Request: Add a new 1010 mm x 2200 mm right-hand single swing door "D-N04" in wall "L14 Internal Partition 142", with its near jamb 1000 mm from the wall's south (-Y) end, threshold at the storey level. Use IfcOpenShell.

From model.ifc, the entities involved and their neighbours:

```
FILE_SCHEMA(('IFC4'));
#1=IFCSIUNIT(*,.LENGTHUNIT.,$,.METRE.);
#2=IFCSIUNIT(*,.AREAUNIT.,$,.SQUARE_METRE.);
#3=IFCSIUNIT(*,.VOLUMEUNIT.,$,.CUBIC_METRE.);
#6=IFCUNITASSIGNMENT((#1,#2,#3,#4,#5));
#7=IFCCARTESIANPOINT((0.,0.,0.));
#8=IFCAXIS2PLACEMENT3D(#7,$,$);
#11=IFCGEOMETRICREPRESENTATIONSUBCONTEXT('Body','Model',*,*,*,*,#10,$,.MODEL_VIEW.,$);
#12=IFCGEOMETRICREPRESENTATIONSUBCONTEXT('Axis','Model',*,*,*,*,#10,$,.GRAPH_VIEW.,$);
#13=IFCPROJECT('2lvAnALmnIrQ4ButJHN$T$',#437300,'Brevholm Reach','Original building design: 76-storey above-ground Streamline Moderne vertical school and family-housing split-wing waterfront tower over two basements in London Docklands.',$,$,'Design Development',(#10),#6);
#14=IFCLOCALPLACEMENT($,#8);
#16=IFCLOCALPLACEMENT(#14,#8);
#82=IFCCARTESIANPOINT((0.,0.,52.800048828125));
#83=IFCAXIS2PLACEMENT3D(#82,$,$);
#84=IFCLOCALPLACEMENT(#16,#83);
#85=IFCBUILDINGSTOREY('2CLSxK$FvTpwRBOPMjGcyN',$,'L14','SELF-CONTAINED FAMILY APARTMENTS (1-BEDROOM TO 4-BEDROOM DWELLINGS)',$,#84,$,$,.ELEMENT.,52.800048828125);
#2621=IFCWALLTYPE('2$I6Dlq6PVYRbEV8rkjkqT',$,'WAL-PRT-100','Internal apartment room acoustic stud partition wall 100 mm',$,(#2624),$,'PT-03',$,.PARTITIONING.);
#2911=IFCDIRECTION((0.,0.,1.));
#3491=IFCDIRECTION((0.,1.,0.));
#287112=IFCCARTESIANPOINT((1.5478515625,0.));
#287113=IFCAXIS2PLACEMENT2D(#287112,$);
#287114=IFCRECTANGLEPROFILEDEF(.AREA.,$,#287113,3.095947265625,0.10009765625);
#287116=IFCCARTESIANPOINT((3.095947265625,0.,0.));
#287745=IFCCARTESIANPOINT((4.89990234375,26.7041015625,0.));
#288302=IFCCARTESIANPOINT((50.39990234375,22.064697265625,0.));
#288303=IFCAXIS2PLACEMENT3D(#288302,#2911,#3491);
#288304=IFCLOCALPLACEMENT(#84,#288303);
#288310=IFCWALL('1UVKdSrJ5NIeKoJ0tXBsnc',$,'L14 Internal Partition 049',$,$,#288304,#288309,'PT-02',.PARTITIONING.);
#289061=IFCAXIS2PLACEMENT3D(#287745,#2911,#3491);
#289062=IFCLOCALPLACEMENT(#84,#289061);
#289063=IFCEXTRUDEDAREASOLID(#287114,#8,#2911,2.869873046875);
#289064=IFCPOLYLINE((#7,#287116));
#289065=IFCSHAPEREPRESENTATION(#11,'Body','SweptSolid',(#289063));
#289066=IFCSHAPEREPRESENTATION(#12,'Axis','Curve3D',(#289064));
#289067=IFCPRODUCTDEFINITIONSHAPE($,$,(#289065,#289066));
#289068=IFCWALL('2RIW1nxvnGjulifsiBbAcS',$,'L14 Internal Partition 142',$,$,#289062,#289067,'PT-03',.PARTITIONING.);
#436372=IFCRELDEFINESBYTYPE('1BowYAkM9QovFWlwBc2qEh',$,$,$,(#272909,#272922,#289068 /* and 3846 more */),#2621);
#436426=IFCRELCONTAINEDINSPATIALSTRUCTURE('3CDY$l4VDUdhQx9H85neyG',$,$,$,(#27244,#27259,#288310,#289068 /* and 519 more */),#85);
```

```python
import numpy as np
import ifcopenshell
import ifcopenshell.api.feature
import ifcopenshell.api.geometry
import ifcopenshell.api.root
import ifcopenshell.api.spatial
import ifcopenshell.geom
import ifcopenshell.util.element
import ifcopenshell.util.placement
import ifcopenshell.util.representation
import ifcopenshell.util.shape
import ifcopenshell.util.unit

model = ifcopenshell.open("model.ifc")
unit_scale = ifcopenshell.util.unit.calculate_unit_scale(model)
settings = ifcopenshell.geom.settings()


def volume(element):
    """Net volume in cubic metres, openings subtracted."""
    shape = ifcopenshell.geom.create_shape(settings, element)
    return ifcopenshell.util.shape.get_volume(shape.geometry)


wall = model.by_guid("2RIW1nxvnGjulifsiBbAcS")
storey = ifcopenshell.util.element.get_container(wall, ifc_class="IfcBuildingStorey")
context = ifcopenshell.util.representation.get_context(model, "Model", "Body", "MODEL_VIEW")
before = volume(wall)

width, height, from_end, sill = 1.01, 2.2, 1, 0.0  # metres

# The wall runs along its own X axis, and the end named is its -X end.
wall_shape = ifcopenshell.geom.create_shape(settings, wall)
x, y, z = ifcopenshell.util.shape.get_vertices(wall_shape.geometry).T
start = x.min() + from_end
face, thickness = float(y.min()), float(y.max() - y.min())
wall_matrix = ifcopenshell.util.placement.get_local_placement(wall.ObjectPlacement)
level = ifcopenshell.util.placement.get_local_placement(storey.ObjectPlacement)[2, 3]


def in_wall(x, y):
    """Placement at x, y metres in the wall's axes, at sill height."""
    matrix = wall_matrix.copy()
    matrix[:, 3] = wall_matrix @ np.array([x / unit_scale, y / unit_scale, 0.0, 1.0])
    matrix[2, 3] = level + sill / unit_scale
    return matrix


# Opening: a box that overshoots both wall faces by 50 mm.
opening = ifcopenshell.api.root.create_entity(model, ifc_class="IfcOpeningElement", predefined_type="OPENING")
box = ifcopenshell.api.geometry.add_wall_representation(
    model, context=context, length=width, height=height, thickness=thickness + 0.1
)
ifcopenshell.api.geometry.assign_representation(model, product=opening, representation=box)
ifcopenshell.api.geometry.edit_object_placement(model, product=opening, matrix=in_wall(start, face - 0.05), is_si=False)
ifcopenshell.api.feature.add_feature(model, feature=opening, element=wall)

door = ifcopenshell.api.root.create_entity(model, ifc_class="IfcDoor", name="D-N04", predefined_type="DOOR")
door.OverallWidth, door.OverallHeight = width / unit_scale, height / unit_scale
door.OperationType = "SINGLE_SWING_RIGHT"
body = ifcopenshell.api.geometry.add_door_representation(
    model,
    context=context,
    overall_width=door.OverallWidth,
    overall_height=door.OverallHeight,
    operation_type="SINGLE_SWING_RIGHT",
    lining_properties={"LiningDepth": thickness / unit_scale, "ThresholdDepth": thickness / unit_scale},
)
ifcopenshell.api.geometry.assign_representation(model, product=door, representation=body)
ifcopenshell.api.spatial.assign_container(model, products=[door], relating_structure=storey)
ifcopenshell.api.feature.add_filling(model, opening=opening, element=door)

# The lining spans the wall, so the door starts at the wall face.
ifcopenshell.api.geometry.edit_object_placement(model, product=door, matrix=in_wall(start, face), is_si=False)

after = volume(wall)

print(f"wall volume {before:.3f} -> {after:.3f} m3")

model.write("model_rev.ifc")
```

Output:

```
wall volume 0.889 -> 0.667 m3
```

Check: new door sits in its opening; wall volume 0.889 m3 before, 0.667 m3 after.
